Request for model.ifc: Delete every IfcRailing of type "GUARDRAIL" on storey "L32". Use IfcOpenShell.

First a look at what the model holds.

```python
import ifcopenshell
import ifcopenshell.util.element

model = ifcopenshell.open("model.ifc")
print(model.schema)
storey = next(s for s in model.by_type("IfcBuildingStorey") if s.Name == "L32")
railings = [e for e in ifcopenshell.util.element.get_decomposition(storey) if e.is_a("IfcRailing")]
seen = {}
for e in railings:
    element_type = ifcopenshell.util.element.get_type(e)
    name = element_type.Name if element_type not in (None, e) else None
    seen[name] = seen.get(name, 0) + 1
for name, count in sorted(seen.items(), key=str):
    print(count, "x", name)
```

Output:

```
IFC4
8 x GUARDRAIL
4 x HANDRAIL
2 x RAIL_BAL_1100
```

```python
import ifcopenshell
import ifcopenshell.api.root
import ifcopenshell.util.element

model = ifcopenshell.open("model.ifc")

storey = next(s for s in model.by_type("IfcBuildingStorey") if s.Name == "L32")
railings = [e for e in ifcopenshell.util.element.get_decomposition(storey) if e.is_a("IfcRailing")]
targets = [e for e in railings if (t := ifcopenshell.util.element.get_type(e)) not in (None, e) and t.Name == "GUARDRAIL"]

for e in targets:
    ifcopenshell.api.root.remove_product(model, product=e)
print(len(targets), "removed")

model.write("model_v2.ifc")
```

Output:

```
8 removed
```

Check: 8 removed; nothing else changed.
